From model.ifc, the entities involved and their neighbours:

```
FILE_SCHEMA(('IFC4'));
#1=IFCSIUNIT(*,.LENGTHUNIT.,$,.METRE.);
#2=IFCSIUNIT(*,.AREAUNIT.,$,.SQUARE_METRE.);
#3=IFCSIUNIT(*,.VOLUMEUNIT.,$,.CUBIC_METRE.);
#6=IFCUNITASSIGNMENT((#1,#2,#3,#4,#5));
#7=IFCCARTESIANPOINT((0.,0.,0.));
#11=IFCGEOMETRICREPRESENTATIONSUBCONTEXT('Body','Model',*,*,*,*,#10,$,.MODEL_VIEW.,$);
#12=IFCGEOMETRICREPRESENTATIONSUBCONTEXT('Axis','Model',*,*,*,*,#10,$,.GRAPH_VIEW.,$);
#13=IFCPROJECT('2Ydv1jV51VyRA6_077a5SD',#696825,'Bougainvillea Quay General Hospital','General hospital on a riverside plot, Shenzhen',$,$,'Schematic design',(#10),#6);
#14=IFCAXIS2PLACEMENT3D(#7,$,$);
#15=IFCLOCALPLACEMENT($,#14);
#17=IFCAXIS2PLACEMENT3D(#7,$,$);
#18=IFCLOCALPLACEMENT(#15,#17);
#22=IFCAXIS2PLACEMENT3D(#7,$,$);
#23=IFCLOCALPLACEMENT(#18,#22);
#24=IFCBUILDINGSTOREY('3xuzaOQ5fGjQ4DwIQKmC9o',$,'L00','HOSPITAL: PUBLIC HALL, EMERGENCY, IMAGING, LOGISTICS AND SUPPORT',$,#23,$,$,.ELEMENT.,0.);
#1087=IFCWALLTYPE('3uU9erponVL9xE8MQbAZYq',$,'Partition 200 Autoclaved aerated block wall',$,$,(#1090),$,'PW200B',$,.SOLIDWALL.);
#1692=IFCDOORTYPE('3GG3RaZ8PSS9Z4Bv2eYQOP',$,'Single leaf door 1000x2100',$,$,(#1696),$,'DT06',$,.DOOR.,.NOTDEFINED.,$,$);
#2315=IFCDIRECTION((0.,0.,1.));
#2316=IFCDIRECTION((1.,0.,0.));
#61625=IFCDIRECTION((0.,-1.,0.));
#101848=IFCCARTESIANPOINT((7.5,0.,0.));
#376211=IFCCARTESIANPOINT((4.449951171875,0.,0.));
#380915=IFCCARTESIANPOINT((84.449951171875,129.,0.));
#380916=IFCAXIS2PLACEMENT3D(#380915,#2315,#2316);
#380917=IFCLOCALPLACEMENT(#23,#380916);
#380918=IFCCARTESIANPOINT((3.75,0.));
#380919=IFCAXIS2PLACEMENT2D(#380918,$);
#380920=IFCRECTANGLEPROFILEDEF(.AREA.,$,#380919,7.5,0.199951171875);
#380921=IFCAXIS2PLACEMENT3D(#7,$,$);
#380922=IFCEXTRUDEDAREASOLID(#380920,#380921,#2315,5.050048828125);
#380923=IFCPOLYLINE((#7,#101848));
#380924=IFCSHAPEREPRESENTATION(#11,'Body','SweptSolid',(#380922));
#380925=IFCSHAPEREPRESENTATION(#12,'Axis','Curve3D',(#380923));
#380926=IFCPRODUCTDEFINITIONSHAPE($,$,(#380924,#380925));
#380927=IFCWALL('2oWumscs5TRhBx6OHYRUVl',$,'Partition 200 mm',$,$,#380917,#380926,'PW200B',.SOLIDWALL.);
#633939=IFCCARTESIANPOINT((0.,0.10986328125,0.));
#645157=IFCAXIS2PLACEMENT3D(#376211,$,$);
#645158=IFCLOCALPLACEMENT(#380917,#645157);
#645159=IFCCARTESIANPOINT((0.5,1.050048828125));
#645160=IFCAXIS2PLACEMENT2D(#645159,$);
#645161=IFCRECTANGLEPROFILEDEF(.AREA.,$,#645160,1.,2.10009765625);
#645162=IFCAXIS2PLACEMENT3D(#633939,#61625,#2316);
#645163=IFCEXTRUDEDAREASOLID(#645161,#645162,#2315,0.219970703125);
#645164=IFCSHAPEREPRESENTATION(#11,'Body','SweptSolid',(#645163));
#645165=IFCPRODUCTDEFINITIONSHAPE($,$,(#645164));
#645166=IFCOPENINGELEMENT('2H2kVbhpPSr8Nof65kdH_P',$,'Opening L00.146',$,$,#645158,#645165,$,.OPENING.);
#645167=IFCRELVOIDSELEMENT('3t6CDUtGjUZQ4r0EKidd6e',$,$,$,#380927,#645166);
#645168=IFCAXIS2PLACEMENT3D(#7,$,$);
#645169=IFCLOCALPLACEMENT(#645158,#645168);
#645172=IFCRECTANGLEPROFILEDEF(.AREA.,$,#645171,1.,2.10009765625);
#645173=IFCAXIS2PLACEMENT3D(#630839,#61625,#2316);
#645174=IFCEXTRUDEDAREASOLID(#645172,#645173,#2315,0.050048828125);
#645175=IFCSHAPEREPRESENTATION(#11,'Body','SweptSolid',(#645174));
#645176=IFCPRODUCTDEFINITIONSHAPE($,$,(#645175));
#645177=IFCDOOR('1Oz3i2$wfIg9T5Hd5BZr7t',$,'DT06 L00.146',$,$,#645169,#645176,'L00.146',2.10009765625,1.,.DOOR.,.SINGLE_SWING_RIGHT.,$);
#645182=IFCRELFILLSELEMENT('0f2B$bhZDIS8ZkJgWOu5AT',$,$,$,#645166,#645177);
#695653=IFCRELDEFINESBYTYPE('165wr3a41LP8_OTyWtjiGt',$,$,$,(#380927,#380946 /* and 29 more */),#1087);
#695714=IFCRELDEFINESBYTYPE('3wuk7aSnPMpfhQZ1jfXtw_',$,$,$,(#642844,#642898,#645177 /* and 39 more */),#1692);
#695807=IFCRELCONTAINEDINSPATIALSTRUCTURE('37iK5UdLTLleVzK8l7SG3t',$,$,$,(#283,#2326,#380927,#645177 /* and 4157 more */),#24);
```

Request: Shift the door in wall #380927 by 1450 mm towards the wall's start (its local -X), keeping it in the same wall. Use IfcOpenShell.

```python
import ifcopenshell
import ifcopenshell.api.geometry
import ifcopenshell.util.placement
import ifcopenshell.util.unit

model = ifcopenshell.open("model.ifc")
unit_scale = ifcopenshell.util.unit.calculate_unit_scale(model)

door = model.by_id(645177)
opening = door.FillsVoids[0].RelatingOpeningElement
wall = opening.VoidsElements[0].RelatingBuildingElement

wall_matrix = ifcopenshell.util.placement.get_local_placement(wall.ObjectPlacement)
shift = wall_matrix[:3, 0] * -1.45 / unit_scale
before = ifcopenshell.util.placement.get_local_placement(door.ObjectPlacement)[:3, 3].copy()

# The door is placed relative to its opening, so it follows when the opening moves.
matrix = ifcopenshell.util.placement.get_local_placement(opening.ObjectPlacement)
matrix[:3, 3] += shift
ifcopenshell.api.geometry.edit_object_placement(
    model, product=opening, matrix=matrix, is_si=False, should_transform_children=True
)

after = ifcopenshell.util.placement.get_local_placement(door.ObjectPlacement)[:3, 3]
print("door moved by", (after - before).round(3) + 0.0)

model.write("model_v2.ifc")
```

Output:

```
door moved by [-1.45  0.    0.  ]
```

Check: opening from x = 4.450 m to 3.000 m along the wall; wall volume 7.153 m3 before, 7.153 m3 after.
